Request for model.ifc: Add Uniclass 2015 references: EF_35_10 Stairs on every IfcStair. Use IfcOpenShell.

First a look at what the model holds.

```python
import ifcopenshell

model = ifcopenshell.open("model.ifc")
print(model.schema)
print("classifications:", [c.Name for c in model.by_type("IfcClassification")])
for ifc_class in ("IfcDoor", "IfcRoof", "IfcStair", "IfcWall", "IfcWindow"):
    print(ifc_class, len(model.by_type(ifc_class)))
```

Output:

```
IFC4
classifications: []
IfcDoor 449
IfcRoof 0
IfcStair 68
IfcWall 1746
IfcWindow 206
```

```python
import ifcopenshell
import ifcopenshell.api.classification

model = ifcopenshell.open("model.ifc")

system = ifcopenshell.api.classification.add_classification(model, classification="Uniclass 2015")

codes = {
    "IfcStair": ("EF_35_10", "Stairs"),
}
for ifc_class, (code, name) in codes.items():
    products = model.by_type(ifc_class)
    ifcopenshell.api.classification.add_reference(
        model, products=products, classification=system, identification=code, name=name
    )
    print(code, len(products))

model.write("model-out.ifc")
```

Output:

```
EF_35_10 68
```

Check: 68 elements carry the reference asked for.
